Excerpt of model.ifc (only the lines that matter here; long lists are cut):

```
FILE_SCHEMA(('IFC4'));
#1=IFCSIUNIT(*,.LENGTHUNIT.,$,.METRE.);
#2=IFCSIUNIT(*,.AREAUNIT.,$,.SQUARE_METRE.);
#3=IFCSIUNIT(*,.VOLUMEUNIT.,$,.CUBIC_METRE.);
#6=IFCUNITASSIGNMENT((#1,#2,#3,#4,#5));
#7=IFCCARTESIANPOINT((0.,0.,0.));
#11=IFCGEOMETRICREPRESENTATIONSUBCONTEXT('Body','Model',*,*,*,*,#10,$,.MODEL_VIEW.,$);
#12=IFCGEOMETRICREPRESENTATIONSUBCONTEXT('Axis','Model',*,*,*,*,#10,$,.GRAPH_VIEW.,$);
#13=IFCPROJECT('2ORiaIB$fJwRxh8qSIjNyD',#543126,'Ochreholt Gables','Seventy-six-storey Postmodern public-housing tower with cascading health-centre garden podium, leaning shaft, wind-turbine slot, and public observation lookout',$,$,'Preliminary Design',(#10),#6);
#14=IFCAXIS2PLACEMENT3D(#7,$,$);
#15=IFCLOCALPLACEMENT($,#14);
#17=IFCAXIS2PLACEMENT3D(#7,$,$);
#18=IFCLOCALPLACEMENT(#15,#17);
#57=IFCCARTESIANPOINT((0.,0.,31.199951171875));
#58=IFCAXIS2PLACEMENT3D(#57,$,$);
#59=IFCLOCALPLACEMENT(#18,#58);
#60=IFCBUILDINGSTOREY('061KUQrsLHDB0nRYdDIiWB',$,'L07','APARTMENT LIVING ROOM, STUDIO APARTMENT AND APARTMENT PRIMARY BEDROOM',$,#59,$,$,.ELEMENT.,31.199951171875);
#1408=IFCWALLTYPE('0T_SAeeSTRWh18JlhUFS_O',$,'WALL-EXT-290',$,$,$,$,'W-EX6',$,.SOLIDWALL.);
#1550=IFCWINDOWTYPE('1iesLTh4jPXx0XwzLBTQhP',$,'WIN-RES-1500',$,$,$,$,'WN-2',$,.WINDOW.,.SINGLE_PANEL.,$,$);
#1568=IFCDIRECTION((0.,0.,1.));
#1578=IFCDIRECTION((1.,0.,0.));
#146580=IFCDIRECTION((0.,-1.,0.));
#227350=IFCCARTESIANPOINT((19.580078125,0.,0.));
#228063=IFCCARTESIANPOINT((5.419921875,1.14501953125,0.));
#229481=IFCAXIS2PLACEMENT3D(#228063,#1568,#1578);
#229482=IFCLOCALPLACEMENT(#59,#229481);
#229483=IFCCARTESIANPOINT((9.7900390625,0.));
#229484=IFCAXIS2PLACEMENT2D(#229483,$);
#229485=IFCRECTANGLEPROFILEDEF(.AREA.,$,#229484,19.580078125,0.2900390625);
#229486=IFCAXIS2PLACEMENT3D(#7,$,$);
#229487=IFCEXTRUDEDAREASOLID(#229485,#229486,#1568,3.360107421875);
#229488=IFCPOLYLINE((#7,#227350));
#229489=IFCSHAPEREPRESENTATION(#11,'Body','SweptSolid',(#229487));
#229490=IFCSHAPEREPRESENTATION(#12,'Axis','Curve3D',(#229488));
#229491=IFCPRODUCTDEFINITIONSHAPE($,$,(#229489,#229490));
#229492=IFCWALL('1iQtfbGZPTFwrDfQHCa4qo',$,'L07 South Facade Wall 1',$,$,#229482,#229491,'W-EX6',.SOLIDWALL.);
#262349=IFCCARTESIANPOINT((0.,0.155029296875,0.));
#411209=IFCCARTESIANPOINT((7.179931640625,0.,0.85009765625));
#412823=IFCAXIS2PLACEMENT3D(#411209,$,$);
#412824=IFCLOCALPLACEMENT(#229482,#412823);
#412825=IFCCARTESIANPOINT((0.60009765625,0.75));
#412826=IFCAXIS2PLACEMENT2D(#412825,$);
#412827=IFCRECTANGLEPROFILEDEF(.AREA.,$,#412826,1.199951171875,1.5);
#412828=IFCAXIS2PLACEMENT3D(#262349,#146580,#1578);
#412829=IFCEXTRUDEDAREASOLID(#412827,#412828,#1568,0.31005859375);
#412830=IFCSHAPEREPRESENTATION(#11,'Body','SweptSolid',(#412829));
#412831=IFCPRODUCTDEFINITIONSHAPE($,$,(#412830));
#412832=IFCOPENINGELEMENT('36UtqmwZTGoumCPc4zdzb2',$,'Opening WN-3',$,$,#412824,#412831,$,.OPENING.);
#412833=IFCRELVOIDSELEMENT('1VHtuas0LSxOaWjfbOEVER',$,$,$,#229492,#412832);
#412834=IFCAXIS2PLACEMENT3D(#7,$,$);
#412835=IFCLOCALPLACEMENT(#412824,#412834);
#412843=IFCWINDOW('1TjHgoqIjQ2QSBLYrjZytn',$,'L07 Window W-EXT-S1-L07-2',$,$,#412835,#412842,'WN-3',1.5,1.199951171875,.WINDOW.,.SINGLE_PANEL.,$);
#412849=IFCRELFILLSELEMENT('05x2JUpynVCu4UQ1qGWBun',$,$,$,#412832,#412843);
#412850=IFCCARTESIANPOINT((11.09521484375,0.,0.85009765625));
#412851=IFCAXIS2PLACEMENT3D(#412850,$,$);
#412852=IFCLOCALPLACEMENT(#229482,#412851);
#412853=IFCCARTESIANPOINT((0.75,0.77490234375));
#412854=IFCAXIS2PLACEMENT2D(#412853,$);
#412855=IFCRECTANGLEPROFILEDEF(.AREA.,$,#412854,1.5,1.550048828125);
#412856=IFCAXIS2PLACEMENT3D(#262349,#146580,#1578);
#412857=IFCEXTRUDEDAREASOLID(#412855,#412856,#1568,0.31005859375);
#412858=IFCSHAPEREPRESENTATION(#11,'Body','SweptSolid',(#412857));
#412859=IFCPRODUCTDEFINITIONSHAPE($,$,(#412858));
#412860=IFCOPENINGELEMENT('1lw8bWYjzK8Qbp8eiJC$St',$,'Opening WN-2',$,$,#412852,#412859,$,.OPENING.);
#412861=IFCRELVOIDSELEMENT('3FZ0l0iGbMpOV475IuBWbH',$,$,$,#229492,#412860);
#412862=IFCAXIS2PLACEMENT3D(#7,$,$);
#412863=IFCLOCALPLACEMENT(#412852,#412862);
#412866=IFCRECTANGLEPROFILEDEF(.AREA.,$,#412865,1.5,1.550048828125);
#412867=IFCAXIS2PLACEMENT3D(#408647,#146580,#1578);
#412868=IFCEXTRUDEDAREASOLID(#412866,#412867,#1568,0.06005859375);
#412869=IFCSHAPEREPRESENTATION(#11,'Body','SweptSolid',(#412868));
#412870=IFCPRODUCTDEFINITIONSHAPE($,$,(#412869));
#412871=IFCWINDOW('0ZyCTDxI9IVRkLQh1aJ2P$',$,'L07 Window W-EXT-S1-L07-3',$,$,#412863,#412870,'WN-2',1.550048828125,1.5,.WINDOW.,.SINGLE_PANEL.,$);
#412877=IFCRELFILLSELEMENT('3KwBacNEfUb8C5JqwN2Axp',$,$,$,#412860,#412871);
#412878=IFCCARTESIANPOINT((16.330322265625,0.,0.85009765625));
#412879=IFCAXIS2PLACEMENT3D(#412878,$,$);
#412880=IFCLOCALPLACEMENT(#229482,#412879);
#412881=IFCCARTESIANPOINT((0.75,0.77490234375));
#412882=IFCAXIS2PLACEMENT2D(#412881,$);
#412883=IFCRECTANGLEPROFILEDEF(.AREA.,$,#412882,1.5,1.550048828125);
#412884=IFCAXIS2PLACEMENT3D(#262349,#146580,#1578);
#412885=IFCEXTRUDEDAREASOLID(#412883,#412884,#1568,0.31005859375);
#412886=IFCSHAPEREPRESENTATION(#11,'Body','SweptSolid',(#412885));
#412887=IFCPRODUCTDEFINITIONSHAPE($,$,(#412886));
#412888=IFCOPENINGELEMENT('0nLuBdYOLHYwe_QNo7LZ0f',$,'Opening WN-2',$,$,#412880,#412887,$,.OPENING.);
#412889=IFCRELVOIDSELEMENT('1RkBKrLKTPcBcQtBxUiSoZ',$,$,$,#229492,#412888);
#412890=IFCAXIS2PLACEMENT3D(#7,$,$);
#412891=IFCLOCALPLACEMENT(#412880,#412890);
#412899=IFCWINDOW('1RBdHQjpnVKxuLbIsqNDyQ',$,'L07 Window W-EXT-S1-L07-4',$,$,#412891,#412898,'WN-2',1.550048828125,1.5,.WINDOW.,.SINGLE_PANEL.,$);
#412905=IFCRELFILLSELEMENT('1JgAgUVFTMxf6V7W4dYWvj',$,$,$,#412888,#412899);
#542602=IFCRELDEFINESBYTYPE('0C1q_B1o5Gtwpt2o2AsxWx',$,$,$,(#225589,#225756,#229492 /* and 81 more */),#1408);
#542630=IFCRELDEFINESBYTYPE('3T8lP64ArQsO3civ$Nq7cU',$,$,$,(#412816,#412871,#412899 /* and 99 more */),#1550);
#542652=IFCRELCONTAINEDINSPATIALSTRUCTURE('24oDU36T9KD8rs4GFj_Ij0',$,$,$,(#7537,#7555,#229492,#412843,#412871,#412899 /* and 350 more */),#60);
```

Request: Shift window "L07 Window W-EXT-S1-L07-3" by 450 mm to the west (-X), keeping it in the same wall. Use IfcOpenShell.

```python
import ifcopenshell
import ifcopenshell.api.geometry
import ifcopenshell.util.placement
import ifcopenshell.util.unit

model = ifcopenshell.open("model.ifc")
unit_scale = ifcopenshell.util.unit.calculate_unit_scale(model)

window = model.by_id(412871)
opening = window.FillsVoids[0].RelatingOpeningElement
wall = opening.VoidsElements[0].RelatingBuildingElement

wall_matrix = ifcopenshell.util.placement.get_local_placement(wall.ObjectPlacement)
shift = wall_matrix[:3, 0] * -0.45 / unit_scale
before = ifcopenshell.util.placement.get_local_placement(window.ObjectPlacement)[:3, 3].copy()

# The window is placed relative to its opening, so it follows when the opening moves.
matrix = ifcopenshell.util.placement.get_local_placement(opening.ObjectPlacement)
matrix[:3, 3] += shift
ifcopenshell.api.geometry.edit_object_placement(
    model, product=opening, matrix=matrix, is_si=False, should_transform_children=True
)

after = ifcopenshell.util.placement.get_local_placement(window.ObjectPlacement)[:3, 3]
print("window moved by", (after - before).round(3) + 0.0)

model.write("model_rev.ifc")
```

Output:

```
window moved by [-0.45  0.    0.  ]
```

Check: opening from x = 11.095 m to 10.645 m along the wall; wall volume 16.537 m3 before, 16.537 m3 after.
